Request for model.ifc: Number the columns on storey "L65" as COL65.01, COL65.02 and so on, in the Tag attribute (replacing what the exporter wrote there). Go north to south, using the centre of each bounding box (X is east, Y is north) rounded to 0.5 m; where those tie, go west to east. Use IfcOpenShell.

First a look at what the model holds.

```python
import ifcopenshell
import ifcopenshell.util.element
import ifcopenshell.util.placement

model = ifcopenshell.open("model.ifc")
print(model.schema)
storey = next(s for s in model.by_type("IfcBuildingStorey") if s.Name == "L65")
columns = [e for e in ifcopenshell.util.element.get_decomposition(storey) if e.is_a("IfcColumn")]
for e in sorted(columns, key=lambda e: e.id()):
    origin = ifcopenshell.util.placement.get_local_placement(e.ObjectPlacement)[:3, 3]
    print(e.id(), e.Tag, e.Name, origin.round(2) + 0.0, sep=" | ")
```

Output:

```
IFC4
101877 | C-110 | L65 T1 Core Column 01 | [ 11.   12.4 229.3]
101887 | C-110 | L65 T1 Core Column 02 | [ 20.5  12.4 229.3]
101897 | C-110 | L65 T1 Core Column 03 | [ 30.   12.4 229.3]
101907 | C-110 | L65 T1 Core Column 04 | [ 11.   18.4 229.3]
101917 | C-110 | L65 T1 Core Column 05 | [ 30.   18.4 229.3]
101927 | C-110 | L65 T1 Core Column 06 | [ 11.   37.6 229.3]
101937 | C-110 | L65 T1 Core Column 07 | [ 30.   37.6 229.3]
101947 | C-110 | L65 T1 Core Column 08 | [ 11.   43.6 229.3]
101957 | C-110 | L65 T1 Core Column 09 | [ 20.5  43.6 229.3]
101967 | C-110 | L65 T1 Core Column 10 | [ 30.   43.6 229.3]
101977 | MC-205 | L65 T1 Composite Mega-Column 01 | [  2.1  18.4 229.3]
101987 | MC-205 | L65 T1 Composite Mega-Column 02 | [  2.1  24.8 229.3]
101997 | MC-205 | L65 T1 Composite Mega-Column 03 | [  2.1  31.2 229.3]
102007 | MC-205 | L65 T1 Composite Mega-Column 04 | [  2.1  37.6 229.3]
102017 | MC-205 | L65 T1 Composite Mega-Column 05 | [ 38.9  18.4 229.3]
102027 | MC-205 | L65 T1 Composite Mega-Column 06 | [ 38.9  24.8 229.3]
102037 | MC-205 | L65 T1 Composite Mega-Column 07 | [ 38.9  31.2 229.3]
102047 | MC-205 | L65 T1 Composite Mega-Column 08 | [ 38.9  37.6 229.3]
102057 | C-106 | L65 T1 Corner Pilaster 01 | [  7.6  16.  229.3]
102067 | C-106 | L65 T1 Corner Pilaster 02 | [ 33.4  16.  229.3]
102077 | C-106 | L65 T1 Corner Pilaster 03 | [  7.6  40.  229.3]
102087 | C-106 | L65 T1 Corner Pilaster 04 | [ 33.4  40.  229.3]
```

```python
import ifcopenshell
import ifcopenshell.geom
import ifcopenshell.util.element
import ifcopenshell.util.shape

model = ifcopenshell.open("model.ifc")
settings = ifcopenshell.geom.settings()
settings.set("use-world-coords", True)


def centre(element):
    shape = ifcopenshell.geom.create_shape(settings, element)
    return ifcopenshell.util.shape.get_bbox_centroid(shape.geometry)


storey = next(s for s in model.by_type("IfcBuildingStorey") if s.Name == "L65")
columns = [e for e in ifcopenshell.util.element.get_decomposition(storey) if e.is_a("IfcColumn")]

# Insertion points can sit at a corner or the storey origin, so sort by the geometry (in metres).
centres = {e: centre(e) for e in columns}
columns.sort(key=lambda e: (-round(centres[e][1] / 0.5), centres[e][0]))

for i, e in enumerate(columns, start=1):
    number = f"COL65.{i:02d}"
    e.Tag = number
    print(e.id(), number)

model.write("model_edited.ifc")
```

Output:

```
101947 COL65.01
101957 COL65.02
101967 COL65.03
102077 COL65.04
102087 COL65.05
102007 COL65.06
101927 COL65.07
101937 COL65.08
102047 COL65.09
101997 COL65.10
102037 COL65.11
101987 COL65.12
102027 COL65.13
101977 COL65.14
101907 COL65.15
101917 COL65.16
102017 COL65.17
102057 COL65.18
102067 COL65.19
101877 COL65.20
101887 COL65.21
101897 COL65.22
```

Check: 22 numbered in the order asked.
